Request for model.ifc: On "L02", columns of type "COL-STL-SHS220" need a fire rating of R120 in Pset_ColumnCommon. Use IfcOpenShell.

First a look at what the model holds.

```python
import ifcopenshell
import ifcopenshell.util.element

model = ifcopenshell.open("model.ifc")
print(model.schema)
storey = next(s for s in model.by_type("IfcBuildingStorey") if s.Name == "L02")
columns = [e for e in ifcopenshell.util.element.get_decomposition(storey) if e.is_a("IfcColumn")]
seen = {}
for e in columns:
    element_type = ifcopenshell.util.element.get_type(e)
    key = (element_type.Name if element_type != e and element_type else None, ifcopenshell.util.element.get_pset(e, "Pset_ColumnCommon", "FireRating"))
    seen[key] = seen.get(key, 0) + 1
for (name, value), count in sorted(seen.items(), key=str):
    print(count, "x", name, "|", value)
```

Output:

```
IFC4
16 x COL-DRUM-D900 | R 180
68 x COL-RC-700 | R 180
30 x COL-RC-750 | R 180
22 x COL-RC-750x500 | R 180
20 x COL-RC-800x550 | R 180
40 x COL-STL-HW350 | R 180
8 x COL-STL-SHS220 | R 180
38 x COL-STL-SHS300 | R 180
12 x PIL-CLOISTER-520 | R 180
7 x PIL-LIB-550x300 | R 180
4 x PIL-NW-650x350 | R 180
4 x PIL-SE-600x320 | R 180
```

```python
import ifcopenshell
import ifcopenshell.api.pset
import ifcopenshell.util.element

model = ifcopenshell.open("model.ifc")

storey = next(s for s in model.by_type("IfcBuildingStorey") if s.Name == "L02")
columns = [e for e in ifcopenshell.util.element.get_decomposition(storey) if e.is_a("IfcColumn")]

count = 0
for e in columns:
    element_type = ifcopenshell.util.element.get_type(e)
    if element_type in (None, e) or element_type.Name != "COL-STL-SHS220":
        continue
    # add_pset returns the element's existing set when there is one.
    pset = ifcopenshell.api.pset.add_pset(model, product=e, name="Pset_ColumnCommon")
    ifcopenshell.api.pset.edit_pset(model, pset=pset, properties={"FireRating": "R120"})
    count += 1

print(count, "columns updated")

model.write("model_rev.ifc")
```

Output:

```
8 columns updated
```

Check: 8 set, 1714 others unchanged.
